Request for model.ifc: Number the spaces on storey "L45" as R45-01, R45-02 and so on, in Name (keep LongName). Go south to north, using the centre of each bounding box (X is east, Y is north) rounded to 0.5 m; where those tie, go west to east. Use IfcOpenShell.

First a look at what the model holds.

```python
import ifcopenshell
import ifcopenshell.util.element
import ifcopenshell.util.placement

model = ifcopenshell.open("model.ifc")
print(model.schema)
storey = next(s for s in model.by_type("IfcBuildingStorey") if s.Name == "L45")
spaces = [e for e in ifcopenshell.util.element.get_decomposition(storey) if e.is_a("IfcSpace")]
for e in sorted(spaces, key=lambda e: e.id()):
    origin = ifcopenshell.util.placement.get_local_placement(e.ObjectPlacement)[:3, 3]
    print(e.id(), e.Name, e.LongName, origin.round(2) + 0.0, sep=" | ")
```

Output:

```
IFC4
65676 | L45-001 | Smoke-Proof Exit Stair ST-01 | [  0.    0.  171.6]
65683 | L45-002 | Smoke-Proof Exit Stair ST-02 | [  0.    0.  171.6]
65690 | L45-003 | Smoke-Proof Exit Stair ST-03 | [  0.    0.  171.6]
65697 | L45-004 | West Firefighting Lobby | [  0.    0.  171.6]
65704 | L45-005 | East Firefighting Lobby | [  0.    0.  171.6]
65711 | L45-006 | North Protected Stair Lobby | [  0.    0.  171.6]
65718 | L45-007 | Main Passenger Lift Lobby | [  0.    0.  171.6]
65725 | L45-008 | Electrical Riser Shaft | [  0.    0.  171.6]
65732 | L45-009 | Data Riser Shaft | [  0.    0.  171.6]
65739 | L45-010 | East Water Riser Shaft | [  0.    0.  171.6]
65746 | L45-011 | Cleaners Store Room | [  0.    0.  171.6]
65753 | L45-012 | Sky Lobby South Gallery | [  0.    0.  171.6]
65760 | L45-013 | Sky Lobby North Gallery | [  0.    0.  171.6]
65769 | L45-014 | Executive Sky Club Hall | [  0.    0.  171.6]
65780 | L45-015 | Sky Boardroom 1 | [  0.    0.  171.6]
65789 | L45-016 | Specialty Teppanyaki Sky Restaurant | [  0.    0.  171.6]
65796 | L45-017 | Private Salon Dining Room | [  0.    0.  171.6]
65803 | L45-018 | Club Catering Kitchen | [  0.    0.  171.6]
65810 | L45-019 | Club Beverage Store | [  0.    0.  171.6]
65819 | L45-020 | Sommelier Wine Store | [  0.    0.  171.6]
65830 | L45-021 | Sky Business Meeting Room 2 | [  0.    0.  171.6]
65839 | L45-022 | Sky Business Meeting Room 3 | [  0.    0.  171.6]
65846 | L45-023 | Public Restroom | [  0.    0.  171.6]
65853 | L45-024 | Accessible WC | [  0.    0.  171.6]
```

```python
import ifcopenshell
import ifcopenshell.geom
import ifcopenshell.util.element
import ifcopenshell.util.shape

model = ifcopenshell.open("model.ifc")
settings = ifcopenshell.geom.settings()
settings.set("use-world-coords", True)


def centre(element):
    shape = ifcopenshell.geom.create_shape(settings, element)
    return ifcopenshell.util.shape.get_bbox_centroid(shape.geometry)


storey = next(s for s in model.by_type("IfcBuildingStorey") if s.Name == "L45")
spaces = [e for e in ifcopenshell.util.element.get_decomposition(storey) if e.is_a("IfcSpace")]

# Insertion points can sit at a corner or the storey origin, so sort by the geometry (in metres).
centres = {e: centre(e) for e in spaces}
spaces.sort(key=lambda e: (round(centres[e][1] / 0.5), centres[e][0]))

for i, e in enumerate(spaces, start=1):
    number = f"R45-{i:02d}"
    e.Name = number
    print(e.id(), number)

model.write("model_rev.ifc")
```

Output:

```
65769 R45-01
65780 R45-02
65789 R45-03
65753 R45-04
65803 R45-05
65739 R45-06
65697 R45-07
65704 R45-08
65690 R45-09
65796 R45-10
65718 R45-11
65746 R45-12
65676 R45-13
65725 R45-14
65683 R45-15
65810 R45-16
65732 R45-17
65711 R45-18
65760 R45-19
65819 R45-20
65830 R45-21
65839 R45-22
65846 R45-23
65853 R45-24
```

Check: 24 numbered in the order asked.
